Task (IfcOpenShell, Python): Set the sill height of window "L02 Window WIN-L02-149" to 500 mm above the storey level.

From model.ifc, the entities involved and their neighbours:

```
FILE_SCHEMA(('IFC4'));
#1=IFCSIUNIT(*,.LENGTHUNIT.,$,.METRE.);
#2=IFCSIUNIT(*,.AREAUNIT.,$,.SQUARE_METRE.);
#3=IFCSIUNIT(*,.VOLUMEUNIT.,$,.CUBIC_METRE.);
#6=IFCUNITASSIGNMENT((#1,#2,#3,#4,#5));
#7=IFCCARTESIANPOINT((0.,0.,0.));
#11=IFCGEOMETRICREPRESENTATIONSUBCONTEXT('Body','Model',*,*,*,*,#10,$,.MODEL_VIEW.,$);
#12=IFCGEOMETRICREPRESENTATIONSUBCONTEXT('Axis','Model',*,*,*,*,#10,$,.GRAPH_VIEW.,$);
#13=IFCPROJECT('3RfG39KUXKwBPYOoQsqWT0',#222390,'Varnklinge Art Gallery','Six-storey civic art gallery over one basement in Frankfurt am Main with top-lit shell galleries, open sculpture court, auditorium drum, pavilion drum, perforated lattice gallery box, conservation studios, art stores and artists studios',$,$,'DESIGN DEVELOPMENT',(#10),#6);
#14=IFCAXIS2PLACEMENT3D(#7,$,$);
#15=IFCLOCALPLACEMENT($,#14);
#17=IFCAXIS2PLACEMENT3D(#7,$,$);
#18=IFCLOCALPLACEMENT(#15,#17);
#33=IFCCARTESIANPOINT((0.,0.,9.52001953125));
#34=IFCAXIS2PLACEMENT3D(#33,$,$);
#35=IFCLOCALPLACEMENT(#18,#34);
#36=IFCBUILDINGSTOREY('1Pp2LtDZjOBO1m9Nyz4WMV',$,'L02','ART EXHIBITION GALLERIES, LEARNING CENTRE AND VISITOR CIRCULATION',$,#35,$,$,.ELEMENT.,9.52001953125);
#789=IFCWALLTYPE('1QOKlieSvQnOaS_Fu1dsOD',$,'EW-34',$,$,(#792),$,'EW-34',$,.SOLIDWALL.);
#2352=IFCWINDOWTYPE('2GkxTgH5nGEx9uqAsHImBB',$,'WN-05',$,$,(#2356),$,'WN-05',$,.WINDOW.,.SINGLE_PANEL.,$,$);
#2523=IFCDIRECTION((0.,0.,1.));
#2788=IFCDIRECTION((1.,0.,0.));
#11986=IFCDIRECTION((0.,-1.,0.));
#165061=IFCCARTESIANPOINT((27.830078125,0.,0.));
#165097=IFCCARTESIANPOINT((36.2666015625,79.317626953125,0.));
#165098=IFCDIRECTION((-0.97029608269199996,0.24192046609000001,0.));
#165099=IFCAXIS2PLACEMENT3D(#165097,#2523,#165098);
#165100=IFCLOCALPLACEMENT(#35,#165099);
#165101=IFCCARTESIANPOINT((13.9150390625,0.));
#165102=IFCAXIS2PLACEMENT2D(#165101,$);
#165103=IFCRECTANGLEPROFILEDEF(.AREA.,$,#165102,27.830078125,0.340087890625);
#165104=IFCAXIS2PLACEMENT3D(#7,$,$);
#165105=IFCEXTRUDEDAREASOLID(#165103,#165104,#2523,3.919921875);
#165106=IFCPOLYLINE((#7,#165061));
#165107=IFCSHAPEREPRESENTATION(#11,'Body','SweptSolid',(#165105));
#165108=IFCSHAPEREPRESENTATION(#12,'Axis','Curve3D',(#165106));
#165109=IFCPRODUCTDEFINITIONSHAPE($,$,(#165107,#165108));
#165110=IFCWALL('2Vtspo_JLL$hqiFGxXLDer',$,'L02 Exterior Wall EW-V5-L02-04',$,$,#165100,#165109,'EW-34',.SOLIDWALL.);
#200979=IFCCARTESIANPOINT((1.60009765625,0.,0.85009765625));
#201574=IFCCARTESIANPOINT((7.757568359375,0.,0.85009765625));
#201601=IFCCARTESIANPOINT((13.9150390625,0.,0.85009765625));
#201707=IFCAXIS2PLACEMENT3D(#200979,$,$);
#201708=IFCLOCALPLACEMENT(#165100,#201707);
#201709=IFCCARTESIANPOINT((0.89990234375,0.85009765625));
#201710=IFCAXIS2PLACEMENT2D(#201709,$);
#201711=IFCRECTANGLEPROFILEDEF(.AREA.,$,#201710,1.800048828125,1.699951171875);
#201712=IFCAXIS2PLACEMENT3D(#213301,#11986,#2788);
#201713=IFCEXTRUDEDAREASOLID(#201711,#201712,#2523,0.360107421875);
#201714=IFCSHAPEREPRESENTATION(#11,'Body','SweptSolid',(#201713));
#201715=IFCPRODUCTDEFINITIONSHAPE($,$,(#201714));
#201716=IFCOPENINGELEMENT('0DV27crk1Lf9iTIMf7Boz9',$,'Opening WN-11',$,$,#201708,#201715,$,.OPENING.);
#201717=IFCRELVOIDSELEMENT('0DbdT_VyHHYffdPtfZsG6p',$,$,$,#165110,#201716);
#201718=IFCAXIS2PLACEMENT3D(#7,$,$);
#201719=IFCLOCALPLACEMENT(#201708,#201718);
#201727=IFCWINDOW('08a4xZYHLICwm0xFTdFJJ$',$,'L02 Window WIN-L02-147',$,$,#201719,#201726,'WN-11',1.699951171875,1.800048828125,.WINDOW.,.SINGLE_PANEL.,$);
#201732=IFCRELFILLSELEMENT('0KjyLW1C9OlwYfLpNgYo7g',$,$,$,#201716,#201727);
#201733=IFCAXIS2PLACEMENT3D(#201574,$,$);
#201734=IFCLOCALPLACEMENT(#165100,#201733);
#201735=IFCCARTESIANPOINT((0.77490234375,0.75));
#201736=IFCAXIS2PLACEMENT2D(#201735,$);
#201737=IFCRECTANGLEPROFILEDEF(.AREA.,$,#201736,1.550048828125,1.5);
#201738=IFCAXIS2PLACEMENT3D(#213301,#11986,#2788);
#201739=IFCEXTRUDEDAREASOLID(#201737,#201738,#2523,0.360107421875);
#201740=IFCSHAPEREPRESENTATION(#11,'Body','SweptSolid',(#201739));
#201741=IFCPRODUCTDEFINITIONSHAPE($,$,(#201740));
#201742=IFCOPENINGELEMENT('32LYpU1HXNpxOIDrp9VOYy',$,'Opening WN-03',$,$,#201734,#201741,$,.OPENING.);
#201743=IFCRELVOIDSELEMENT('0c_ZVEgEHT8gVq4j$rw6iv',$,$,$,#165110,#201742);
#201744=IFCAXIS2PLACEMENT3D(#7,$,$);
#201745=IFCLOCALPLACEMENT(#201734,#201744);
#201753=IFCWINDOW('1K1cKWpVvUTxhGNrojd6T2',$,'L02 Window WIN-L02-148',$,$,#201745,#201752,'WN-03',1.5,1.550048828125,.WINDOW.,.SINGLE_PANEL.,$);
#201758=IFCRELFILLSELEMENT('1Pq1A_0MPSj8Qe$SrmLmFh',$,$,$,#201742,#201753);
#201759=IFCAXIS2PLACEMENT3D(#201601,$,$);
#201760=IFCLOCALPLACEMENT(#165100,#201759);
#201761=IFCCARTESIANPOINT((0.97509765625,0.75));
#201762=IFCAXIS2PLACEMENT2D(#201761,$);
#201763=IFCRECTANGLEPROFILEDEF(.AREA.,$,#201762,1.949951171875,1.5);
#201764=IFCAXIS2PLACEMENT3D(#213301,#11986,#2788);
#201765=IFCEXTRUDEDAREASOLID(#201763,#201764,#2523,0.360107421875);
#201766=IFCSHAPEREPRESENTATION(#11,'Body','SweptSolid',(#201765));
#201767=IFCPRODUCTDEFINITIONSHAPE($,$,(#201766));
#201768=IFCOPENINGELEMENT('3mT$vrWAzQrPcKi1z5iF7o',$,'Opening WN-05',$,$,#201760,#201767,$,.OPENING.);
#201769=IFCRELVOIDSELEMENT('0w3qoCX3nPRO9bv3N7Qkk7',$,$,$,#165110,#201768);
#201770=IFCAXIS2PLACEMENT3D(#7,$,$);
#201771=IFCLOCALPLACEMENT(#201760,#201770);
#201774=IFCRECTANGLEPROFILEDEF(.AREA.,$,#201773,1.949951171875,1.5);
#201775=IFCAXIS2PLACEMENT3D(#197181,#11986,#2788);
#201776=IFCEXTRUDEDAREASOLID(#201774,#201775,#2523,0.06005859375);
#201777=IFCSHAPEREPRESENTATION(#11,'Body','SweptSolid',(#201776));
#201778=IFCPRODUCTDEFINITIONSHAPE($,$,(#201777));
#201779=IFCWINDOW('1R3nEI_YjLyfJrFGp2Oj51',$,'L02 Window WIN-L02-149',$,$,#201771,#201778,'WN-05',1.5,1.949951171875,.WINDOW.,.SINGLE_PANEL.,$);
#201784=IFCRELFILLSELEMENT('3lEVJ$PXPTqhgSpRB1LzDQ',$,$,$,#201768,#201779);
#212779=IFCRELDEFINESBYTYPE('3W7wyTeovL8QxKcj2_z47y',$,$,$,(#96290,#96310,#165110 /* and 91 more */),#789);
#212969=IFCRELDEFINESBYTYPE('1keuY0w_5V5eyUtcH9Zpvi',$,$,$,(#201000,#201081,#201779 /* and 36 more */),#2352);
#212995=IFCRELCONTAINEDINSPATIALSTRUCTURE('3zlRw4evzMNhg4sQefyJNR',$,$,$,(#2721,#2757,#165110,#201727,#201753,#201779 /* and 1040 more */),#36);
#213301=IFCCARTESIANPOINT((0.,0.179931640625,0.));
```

```python
import numpy as np
import ifcopenshell
import ifcopenshell.api.geometry
import ifcopenshell.geom
import ifcopenshell.util.element
import ifcopenshell.util.placement
import ifcopenshell.util.shape
import ifcopenshell.util.unit

model = ifcopenshell.open("model.ifc")
unit_scale = ifcopenshell.util.unit.calculate_unit_scale(model)

window = model.by_guid("1R3nEI_YjLyfJrFGp2Oj51")
opening = window.FillsVoids[0].RelatingOpeningElement
storey = ifcopenshell.util.element.get_container(window, ifc_class="IfcBuildingStorey")
level = ifcopenshell.util.placement.get_local_placement(storey.ObjectPlacement)[2, 3]

# The opening's origin need not be at the sill, so measure its lowest point.
shape = ifcopenshell.geom.create_shape(ifcopenshell.geom.settings(), opening)
bottom = ifcopenshell.util.shape.get_shape_bottom_elevation(shape, shape.geometry) / unit_scale
dz = level + 0.5 / unit_scale - bottom

shift = np.array([0.0, 0.0, dz])
# The window is placed relative to its opening, so it follows when the opening moves.
matrix = ifcopenshell.util.placement.get_local_placement(opening.ObjectPlacement)
matrix[:3, 3] += shift
ifcopenshell.api.geometry.edit_object_placement(
    model, product=opening, matrix=matrix, is_si=False, should_transform_children=True
)

print(f"moved by {dz * unit_scale:+.3f} m")

model.write("model-out.ifc")
```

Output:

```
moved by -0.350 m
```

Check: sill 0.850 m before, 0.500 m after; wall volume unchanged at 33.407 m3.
